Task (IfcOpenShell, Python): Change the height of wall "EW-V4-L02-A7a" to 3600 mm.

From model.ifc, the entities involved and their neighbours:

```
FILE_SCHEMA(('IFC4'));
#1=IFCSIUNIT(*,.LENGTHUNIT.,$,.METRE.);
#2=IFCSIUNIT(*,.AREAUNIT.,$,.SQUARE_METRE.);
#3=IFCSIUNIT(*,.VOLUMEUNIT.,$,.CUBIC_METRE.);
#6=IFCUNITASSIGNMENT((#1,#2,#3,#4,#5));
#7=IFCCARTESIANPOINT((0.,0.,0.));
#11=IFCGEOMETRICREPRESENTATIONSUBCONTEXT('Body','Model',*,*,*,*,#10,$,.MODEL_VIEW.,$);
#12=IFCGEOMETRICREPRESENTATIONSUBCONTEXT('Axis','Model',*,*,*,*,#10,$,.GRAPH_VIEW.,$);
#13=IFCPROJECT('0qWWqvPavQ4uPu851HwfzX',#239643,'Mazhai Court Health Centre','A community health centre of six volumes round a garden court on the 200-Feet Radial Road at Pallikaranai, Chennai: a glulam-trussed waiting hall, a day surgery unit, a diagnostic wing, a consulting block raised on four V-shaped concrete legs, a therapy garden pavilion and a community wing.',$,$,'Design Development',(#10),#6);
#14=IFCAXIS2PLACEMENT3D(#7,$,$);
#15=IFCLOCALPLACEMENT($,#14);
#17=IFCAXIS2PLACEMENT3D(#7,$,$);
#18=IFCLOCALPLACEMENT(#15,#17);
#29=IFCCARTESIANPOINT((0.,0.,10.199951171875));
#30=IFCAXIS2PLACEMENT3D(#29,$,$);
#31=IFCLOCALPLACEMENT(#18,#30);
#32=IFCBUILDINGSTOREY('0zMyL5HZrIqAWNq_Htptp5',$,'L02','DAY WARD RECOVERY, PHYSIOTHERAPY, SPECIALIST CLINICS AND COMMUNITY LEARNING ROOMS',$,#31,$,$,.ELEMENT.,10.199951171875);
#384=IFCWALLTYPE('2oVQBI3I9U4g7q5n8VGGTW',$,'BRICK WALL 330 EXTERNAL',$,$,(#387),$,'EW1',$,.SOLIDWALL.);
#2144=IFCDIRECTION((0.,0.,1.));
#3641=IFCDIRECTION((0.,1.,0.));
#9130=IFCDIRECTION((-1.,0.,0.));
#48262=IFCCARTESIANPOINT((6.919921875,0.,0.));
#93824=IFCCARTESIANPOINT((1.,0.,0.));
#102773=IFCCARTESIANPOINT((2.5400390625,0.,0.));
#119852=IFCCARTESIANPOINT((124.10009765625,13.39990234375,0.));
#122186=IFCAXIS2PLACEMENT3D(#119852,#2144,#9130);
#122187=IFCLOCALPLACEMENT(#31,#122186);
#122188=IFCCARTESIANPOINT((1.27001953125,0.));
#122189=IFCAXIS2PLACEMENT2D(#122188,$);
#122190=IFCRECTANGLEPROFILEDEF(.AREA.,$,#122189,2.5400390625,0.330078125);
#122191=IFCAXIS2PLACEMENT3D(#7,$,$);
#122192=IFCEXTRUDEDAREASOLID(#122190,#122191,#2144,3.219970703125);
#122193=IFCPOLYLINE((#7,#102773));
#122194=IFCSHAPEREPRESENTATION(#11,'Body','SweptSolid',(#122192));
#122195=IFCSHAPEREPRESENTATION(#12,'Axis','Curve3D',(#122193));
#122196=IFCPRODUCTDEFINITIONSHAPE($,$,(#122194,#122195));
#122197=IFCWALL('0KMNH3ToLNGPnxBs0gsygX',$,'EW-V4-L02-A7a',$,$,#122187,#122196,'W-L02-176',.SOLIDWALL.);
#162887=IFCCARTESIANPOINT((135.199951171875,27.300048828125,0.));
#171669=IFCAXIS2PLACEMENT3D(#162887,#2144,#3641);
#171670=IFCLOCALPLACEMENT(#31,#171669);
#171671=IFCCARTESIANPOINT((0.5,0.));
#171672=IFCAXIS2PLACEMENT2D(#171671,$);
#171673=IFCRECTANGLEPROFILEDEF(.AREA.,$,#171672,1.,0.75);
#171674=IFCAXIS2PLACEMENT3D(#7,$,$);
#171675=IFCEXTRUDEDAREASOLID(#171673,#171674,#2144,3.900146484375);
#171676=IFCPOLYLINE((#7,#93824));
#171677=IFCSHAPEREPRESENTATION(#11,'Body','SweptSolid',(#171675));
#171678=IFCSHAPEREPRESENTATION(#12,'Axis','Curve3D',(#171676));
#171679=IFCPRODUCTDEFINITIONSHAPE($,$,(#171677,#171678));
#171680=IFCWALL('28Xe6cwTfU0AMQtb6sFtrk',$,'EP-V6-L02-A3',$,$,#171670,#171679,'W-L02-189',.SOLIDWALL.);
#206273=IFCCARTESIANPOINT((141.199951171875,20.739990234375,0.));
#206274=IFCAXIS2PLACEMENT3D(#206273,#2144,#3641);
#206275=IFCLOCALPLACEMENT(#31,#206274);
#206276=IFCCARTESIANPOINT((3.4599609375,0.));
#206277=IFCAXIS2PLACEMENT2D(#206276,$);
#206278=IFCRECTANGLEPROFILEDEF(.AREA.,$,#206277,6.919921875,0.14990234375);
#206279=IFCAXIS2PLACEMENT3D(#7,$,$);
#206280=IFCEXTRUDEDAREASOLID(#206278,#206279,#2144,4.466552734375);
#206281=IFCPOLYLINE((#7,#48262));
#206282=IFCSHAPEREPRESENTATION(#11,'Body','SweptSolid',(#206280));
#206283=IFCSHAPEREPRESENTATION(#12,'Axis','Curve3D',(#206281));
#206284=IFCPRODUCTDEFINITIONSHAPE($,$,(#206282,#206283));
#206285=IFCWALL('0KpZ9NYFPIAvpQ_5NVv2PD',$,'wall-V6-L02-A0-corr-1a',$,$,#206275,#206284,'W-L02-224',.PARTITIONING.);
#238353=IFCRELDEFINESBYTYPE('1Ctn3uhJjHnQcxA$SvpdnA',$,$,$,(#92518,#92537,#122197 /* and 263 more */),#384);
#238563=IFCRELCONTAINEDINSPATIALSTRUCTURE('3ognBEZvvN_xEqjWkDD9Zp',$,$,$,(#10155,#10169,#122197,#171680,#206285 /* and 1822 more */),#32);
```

```python
import ifcopenshell
import ifcopenshell.geom
import ifcopenshell.util.representation
import ifcopenshell.util.shape
import ifcopenshell.util.unit

model = ifcopenshell.open("model.ifc")
unit_scale = ifcopenshell.util.unit.calculate_unit_scale(model)
settings = ifcopenshell.geom.settings()


def volume(element):
    """Net volume in cubic metres, openings subtracted."""
    shape = ifcopenshell.geom.create_shape(settings, element)
    return ifcopenshell.util.shape.get_volume(shape.geometry)


wall = model.by_guid("0KMNH3ToLNGPnxBs0gsygX")
before = volume(wall)

body = ifcopenshell.util.representation.get_representation(wall, "Model", "Body")
solid = body.Items[0]
old_height = solid.Depth
solid.Depth = 3.6 / unit_scale
after = volume(wall)

print(f"height {old_height:g} -> {solid.Depth:g}, volume {before:.3f} -> {after:.3f} m3")

model.write("model_v2.ifc")
```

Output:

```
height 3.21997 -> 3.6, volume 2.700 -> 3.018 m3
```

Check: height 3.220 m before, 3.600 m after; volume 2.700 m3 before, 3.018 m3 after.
